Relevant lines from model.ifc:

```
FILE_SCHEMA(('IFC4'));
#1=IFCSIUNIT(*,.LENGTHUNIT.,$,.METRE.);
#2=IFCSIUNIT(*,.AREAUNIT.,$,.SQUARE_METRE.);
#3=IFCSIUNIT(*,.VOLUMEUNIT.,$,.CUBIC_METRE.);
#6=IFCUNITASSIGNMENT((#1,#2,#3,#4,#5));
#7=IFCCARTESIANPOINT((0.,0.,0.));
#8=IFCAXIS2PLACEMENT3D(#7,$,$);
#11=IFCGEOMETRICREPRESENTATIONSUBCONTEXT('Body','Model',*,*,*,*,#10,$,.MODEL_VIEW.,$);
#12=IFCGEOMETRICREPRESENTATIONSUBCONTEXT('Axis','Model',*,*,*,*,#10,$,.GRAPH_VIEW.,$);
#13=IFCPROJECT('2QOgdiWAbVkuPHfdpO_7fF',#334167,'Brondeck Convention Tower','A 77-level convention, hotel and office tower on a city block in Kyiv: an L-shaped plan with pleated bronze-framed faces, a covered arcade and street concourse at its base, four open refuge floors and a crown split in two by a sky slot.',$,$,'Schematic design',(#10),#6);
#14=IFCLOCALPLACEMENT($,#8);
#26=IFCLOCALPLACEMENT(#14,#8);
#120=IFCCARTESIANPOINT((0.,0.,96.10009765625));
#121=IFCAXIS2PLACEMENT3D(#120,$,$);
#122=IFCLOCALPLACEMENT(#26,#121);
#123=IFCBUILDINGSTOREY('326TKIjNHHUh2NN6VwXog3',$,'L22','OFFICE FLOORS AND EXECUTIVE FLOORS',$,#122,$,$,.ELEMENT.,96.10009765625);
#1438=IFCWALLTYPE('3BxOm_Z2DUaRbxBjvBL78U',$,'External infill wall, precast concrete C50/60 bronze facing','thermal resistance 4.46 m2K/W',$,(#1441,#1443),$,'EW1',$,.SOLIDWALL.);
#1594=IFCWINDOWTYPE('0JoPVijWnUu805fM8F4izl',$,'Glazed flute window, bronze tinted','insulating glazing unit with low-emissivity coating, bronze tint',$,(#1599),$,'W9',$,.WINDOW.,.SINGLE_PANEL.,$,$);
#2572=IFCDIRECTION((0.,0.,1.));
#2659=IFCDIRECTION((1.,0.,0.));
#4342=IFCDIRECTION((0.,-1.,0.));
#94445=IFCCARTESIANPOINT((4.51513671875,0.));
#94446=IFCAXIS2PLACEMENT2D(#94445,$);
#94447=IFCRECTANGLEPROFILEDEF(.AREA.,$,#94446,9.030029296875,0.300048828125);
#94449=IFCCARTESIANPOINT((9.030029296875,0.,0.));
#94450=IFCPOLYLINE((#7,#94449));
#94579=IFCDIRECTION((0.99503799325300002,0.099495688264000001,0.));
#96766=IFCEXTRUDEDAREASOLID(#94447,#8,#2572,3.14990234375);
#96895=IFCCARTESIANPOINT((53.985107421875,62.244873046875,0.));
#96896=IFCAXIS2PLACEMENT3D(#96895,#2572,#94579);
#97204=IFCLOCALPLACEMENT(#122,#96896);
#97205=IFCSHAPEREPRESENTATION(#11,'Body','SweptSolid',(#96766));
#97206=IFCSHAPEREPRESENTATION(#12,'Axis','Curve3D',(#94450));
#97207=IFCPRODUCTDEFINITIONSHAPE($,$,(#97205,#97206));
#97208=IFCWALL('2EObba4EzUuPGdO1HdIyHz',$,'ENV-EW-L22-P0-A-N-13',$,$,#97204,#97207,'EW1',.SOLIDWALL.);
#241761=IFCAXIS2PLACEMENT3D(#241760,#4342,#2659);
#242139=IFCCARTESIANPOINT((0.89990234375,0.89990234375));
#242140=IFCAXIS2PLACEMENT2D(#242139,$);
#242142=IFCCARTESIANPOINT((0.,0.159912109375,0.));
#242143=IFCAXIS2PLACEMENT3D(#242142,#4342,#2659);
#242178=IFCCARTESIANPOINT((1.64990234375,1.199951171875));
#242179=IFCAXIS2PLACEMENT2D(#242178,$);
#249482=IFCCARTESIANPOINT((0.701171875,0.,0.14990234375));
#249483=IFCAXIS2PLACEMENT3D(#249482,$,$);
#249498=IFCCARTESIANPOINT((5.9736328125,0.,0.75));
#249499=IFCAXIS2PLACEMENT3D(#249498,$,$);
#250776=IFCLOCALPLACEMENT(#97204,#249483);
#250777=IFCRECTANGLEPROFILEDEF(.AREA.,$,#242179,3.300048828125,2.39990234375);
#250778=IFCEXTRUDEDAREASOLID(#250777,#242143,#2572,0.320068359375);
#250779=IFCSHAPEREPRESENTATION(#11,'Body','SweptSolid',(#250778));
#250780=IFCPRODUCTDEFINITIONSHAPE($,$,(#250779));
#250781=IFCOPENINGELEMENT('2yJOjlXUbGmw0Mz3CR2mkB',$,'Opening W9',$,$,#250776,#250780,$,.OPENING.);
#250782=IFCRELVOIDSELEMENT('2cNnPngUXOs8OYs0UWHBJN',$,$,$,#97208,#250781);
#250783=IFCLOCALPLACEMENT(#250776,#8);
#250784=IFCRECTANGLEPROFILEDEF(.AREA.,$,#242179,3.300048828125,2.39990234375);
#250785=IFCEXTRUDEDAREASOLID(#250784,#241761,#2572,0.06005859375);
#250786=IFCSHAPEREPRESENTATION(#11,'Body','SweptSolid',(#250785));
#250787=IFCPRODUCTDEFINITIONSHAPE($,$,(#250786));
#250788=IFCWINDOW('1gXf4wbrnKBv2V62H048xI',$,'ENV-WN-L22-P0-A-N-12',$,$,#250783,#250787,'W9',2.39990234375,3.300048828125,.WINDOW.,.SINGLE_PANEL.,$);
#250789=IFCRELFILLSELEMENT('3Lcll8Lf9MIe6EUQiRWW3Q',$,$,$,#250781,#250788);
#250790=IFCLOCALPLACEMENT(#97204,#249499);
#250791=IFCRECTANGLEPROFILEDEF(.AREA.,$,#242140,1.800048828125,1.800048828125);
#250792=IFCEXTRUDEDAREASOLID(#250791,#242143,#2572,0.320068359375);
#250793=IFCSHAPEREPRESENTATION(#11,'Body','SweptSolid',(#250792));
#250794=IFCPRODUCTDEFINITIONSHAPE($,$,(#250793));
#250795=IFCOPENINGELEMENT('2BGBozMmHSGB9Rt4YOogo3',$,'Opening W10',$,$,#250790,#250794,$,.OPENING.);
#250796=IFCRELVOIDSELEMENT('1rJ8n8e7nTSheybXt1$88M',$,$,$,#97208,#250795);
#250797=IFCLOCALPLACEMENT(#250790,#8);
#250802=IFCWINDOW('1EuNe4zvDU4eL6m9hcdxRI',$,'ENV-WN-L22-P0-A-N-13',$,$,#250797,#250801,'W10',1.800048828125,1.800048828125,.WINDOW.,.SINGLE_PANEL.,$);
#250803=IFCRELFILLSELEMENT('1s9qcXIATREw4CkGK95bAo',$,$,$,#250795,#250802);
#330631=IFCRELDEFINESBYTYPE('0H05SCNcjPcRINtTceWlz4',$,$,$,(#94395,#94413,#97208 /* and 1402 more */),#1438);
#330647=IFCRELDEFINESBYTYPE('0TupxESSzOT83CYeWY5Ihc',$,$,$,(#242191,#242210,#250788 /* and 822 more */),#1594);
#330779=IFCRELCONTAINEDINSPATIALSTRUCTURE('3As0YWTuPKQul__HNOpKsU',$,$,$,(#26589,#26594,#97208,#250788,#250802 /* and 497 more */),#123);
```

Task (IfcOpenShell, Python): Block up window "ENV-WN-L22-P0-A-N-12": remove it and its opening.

```python
import ifcopenshell
import ifcopenshell.api.feature
import ifcopenshell.api.root
import ifcopenshell.geom
import ifcopenshell.util.shape

model = ifcopenshell.open("model.ifc")
settings = ifcopenshell.geom.settings()


def volume(element):
    """Net volume in cubic metres, openings subtracted."""
    shape = ifcopenshell.geom.create_shape(settings, element)
    return ifcopenshell.util.shape.get_volume(shape.geometry)


window = model.by_guid("1gXf4wbrnKBv2V62H048xI")
opening = window.FillsVoids[0].RelatingOpeningElement
wall = opening.VoidsElements[0].RelatingBuildingElement
before = volume(wall)

ifcopenshell.api.root.remove_product(model, product=window)
ifcopenshell.api.feature.remove_feature(model, feature=opening)

after = volume(wall)

print(f"wall volume {before:.3f} -> {after:.3f} m3")

model.write("model-out.ifc")
```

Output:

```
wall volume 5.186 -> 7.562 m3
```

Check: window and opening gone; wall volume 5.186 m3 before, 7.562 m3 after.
